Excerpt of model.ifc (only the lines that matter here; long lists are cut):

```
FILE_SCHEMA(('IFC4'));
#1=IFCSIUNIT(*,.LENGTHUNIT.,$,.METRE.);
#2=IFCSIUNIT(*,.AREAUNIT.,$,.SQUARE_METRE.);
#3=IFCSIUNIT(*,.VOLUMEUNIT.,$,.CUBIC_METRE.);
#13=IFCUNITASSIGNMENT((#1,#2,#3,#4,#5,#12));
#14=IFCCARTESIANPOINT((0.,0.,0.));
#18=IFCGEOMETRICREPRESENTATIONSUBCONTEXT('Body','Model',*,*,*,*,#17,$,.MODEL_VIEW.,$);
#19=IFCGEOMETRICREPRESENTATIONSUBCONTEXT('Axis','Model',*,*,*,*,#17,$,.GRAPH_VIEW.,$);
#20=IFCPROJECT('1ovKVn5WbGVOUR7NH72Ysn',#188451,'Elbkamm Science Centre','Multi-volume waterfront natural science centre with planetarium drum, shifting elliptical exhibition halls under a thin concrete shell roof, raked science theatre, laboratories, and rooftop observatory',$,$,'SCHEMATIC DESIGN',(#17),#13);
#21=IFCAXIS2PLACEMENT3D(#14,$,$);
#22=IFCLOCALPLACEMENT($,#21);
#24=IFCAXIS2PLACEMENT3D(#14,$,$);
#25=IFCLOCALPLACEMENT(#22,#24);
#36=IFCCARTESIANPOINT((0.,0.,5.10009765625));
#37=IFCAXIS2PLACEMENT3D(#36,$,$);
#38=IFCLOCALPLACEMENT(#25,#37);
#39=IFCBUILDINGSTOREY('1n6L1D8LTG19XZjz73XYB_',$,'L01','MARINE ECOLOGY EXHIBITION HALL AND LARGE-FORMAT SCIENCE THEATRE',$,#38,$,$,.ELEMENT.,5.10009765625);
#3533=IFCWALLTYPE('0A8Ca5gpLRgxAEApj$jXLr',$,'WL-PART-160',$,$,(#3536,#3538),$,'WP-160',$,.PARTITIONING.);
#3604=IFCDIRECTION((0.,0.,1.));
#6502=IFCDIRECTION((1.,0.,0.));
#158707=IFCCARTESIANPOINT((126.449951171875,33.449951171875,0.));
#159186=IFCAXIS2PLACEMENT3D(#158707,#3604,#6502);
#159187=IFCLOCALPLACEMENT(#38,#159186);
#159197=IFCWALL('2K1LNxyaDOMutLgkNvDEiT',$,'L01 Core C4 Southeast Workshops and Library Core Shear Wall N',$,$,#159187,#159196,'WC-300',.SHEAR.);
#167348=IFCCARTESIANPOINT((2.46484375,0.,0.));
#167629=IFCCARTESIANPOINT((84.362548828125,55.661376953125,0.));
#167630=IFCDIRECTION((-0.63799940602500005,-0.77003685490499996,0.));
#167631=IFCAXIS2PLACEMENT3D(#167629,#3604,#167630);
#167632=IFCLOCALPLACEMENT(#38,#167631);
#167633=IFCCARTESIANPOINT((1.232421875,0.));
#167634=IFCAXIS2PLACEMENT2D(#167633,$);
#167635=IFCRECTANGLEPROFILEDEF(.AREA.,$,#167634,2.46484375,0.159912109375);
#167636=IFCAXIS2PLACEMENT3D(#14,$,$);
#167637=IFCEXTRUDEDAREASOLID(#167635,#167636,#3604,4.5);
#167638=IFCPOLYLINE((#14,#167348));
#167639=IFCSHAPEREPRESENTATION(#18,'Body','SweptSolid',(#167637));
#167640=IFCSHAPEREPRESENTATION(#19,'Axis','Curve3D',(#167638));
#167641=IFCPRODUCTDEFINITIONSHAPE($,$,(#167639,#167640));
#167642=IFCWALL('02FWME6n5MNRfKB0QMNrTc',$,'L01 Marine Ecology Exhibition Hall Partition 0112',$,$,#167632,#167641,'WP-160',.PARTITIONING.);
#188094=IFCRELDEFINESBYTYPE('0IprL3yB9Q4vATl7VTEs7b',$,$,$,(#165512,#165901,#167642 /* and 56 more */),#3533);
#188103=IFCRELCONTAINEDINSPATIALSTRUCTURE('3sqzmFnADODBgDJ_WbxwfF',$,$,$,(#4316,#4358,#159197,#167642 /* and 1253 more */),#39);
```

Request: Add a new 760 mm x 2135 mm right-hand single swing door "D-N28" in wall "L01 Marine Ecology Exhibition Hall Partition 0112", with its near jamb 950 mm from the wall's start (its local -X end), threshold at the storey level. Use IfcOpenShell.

```python
import numpy as np
import ifcopenshell
import ifcopenshell.api.feature
import ifcopenshell.api.geometry
import ifcopenshell.api.root
import ifcopenshell.api.spatial
import ifcopenshell.geom
import ifcopenshell.util.element
import ifcopenshell.util.placement
import ifcopenshell.util.representation
import ifcopenshell.util.shape
import ifcopenshell.util.unit

model = ifcopenshell.open("model.ifc")
unit_scale = ifcopenshell.util.unit.calculate_unit_scale(model)
settings = ifcopenshell.geom.settings()


def volume(element):
    """Net volume in cubic metres, openings subtracted."""
    shape = ifcopenshell.geom.create_shape(settings, element)
    return ifcopenshell.util.shape.get_volume(shape.geometry)


wall = model.by_guid("02FWME6n5MNRfKB0QMNrTc")
storey = ifcopenshell.util.element.get_container(wall, ifc_class="IfcBuildingStorey")
context = ifcopenshell.util.representation.get_context(model, "Model", "Body", "MODEL_VIEW")
before = volume(wall)

width, height, from_end, sill = 0.76, 2.135, 0.95, 0.0  # metres

# The wall runs along its own X axis, and the end named is its -X end.
wall_shape = ifcopenshell.geom.create_shape(settings, wall)
x, y, z = ifcopenshell.util.shape.get_vertices(wall_shape.geometry).T
start = x.min() + from_end
face, thickness = float(y.min()), float(y.max() - y.min())
wall_matrix = ifcopenshell.util.placement.get_local_placement(wall.ObjectPlacement)
level = ifcopenshell.util.placement.get_local_placement(storey.ObjectPlacement)[2, 3]


def in_wall(x, y):
    """Placement at x, y metres in the wall's axes, at sill height."""
    matrix = wall_matrix.copy()
    matrix[:, 3] = wall_matrix @ np.array([x / unit_scale, y / unit_scale, 0.0, 1.0])
    matrix[2, 3] = level + sill / unit_scale
    return matrix


# Opening: a box that overshoots both wall faces by 50 mm.
opening = ifcopenshell.api.root.create_entity(model, ifc_class="IfcOpeningElement", predefined_type="OPENING")
box = ifcopenshell.api.geometry.add_wall_representation(
    model, context=context, length=width, height=height, thickness=thickness + 0.1
)
ifcopenshell.api.geometry.assign_representation(model, product=opening, representation=box)
ifcopenshell.api.geometry.edit_object_placement(model, product=opening, matrix=in_wall(start, face - 0.05), is_si=False)
ifcopenshell.api.feature.add_feature(model, feature=opening, element=wall)

door = ifcopenshell.api.root.create_entity(model, ifc_class="IfcDoor", name="D-N28", predefined_type="DOOR")
door.OverallWidth, door.OverallHeight = width / unit_scale, height / unit_scale
door.OperationType = "SINGLE_SWING_RIGHT"
body = ifcopenshell.api.geometry.add_door_representation(
    model,
    context=context,
    overall_width=door.OverallWidth,
    overall_height=door.OverallHeight,
    operation_type="SINGLE_SWING_RIGHT",
    lining_properties={"LiningDepth": thickness / unit_scale, "ThresholdDepth": thickness / unit_scale},
)
ifcopenshell.api.geometry.assign_representation(model, product=door, representation=body)
ifcopenshell.api.spatial.assign_container(model, products=[door], relating_structure=storey)
ifcopenshell.api.feature.add_filling(model, opening=opening, element=door)

# The lining spans the wall, so the door starts at the wall face.
ifcopenshell.api.geometry.edit_object_placement(model, product=door, matrix=in_wall(start, face), is_si=False)

after = volume(wall)

print(f"wall volume {before:.3f} -> {after:.3f} m3")

model.write("model_rev.ifc")
```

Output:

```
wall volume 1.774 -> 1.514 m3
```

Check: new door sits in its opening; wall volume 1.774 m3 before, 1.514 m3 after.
